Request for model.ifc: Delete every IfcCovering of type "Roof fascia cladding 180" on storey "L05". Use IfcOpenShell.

First a look at what the model holds.

```python
import ifcopenshell
import ifcopenshell.util.element

model = ifcopenshell.open("model.ifc")
print(model.schema)
storey = next(s for s in model.by_type("IfcBuildingStorey") if s.Name == "L05")
coverings = [e for e in ifcopenshell.util.element.get_decomposition(storey) if e.is_a("IfcCovering")]
seen = {}
for e in coverings:
    element_type = ifcopenshell.util.element.get_type(e)
    name = element_type.Name if element_type not in (None, e) else None
    seen[name] = seen.get(name, 0) + 1
for name, count in sorted(seen.items(), key=str):
    print(count, "x", name)
```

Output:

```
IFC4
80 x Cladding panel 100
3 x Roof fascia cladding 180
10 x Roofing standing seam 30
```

```python
import ifcopenshell
import ifcopenshell.api.root
import ifcopenshell.util.element

model = ifcopenshell.open("model.ifc")

storey = next(s for s in model.by_type("IfcBuildingStorey") if s.Name == "L05")
coverings = [e for e in ifcopenshell.util.element.get_decomposition(storey) if e.is_a("IfcCovering")]
targets = [e for e in coverings if (t := ifcopenshell.util.element.get_type(e)) not in (None, e) and t.Name == "Roof fascia cladding 180"]

for e in targets:
    ifcopenshell.api.root.remove_product(model, product=e)
print(len(targets), "removed")

model.write("model_updated.ifc")
```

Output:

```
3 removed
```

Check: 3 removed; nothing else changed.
